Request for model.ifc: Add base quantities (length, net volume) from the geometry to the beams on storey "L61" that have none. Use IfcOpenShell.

First a look at what the model holds.

```python
import ifcopenshell
import ifcopenshell.util.element
import ifcopenshell.util.unit

model = ifcopenshell.open("model.ifc")
print(model.schema)
for unit_type in ("LENGTHUNIT", "AREAUNIT", "VOLUMEUNIT"):
    print(unit_type, ifcopenshell.util.unit.calculate_unit_scale(model, unit_type))
storey = next(s for s in model.by_type("IfcBuildingStorey") if s.Name == "L61")
beams = [e for e in ifcopenshell.util.element.get_decomposition(storey) if e.is_a("IfcBeam")]
for e in sorted(beams, key=lambda e: e.id()):
    print(e.id(), e.is_a(), e.Name, list(ifcopenshell.util.element.get_psets(e, qtos_only=True)), sep=" | ")
```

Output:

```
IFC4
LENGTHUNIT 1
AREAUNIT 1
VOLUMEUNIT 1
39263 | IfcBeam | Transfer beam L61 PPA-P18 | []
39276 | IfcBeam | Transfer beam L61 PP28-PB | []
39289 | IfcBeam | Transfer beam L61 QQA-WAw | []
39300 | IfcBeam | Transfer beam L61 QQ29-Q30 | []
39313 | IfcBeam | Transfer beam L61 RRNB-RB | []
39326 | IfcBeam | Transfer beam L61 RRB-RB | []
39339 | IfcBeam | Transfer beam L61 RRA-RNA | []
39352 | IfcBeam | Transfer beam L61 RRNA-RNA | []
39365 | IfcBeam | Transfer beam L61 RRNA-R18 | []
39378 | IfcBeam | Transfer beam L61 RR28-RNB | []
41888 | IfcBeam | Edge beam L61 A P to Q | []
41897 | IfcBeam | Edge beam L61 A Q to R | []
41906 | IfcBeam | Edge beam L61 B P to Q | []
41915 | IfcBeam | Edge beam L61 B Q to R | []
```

```python
import ifcopenshell
import ifcopenshell.api.pset
import ifcopenshell.geom
import ifcopenshell.util.element
import ifcopenshell.util.shape
import ifcopenshell.util.unit

model = ifcopenshell.open("model.ifc")
unit_scale = ifcopenshell.util.unit.calculate_unit_scale(model)
volume_scale = ifcopenshell.util.unit.calculate_unit_scale(model, "VOLUMEUNIT")
settings = ifcopenshell.geom.settings()

storey = next(s for s in model.by_type("IfcBuildingStorey") if s.Name == "L61")
beams = [e for e in ifcopenshell.util.element.get_decomposition(storey) if e.is_a("IfcBeam")]

for e in sorted(beams, key=lambda e: e.id()):
    if ifcopenshell.util.element.get_psets(e, qtos_only=True, should_inherit=False):
        continue
    # Geometry comes back in metres, in the element's own axes.
    shape = ifcopenshell.geom.create_shape(settings, e)
    values = {
        "Length": ifcopenshell.util.shape.get_max_xyz(shape.geometry) / unit_scale,
        "NetVolume": ifcopenshell.util.shape.get_volume(shape.geometry) / volume_scale,
    }
    qto = ifcopenshell.api.pset.add_qto(model, product=e, name="Qto_BeamBaseQuantities")
    ifcopenshell.api.pset.edit_qto(model, qto=qto, properties=values)
    print(e.id(), {k: round(v, 3) for k, v in values.items()})

model.write("model_rev.ifc")
```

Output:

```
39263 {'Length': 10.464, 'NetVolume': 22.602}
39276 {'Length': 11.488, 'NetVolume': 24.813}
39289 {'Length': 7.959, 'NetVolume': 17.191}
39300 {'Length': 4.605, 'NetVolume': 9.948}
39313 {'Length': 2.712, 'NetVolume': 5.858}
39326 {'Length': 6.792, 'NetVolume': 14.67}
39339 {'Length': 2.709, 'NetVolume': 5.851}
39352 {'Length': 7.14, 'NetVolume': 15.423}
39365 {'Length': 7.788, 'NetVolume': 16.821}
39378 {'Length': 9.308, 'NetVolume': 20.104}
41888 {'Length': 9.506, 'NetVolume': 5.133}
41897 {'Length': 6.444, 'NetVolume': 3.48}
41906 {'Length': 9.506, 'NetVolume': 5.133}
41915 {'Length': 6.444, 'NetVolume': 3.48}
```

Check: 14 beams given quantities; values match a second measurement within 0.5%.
